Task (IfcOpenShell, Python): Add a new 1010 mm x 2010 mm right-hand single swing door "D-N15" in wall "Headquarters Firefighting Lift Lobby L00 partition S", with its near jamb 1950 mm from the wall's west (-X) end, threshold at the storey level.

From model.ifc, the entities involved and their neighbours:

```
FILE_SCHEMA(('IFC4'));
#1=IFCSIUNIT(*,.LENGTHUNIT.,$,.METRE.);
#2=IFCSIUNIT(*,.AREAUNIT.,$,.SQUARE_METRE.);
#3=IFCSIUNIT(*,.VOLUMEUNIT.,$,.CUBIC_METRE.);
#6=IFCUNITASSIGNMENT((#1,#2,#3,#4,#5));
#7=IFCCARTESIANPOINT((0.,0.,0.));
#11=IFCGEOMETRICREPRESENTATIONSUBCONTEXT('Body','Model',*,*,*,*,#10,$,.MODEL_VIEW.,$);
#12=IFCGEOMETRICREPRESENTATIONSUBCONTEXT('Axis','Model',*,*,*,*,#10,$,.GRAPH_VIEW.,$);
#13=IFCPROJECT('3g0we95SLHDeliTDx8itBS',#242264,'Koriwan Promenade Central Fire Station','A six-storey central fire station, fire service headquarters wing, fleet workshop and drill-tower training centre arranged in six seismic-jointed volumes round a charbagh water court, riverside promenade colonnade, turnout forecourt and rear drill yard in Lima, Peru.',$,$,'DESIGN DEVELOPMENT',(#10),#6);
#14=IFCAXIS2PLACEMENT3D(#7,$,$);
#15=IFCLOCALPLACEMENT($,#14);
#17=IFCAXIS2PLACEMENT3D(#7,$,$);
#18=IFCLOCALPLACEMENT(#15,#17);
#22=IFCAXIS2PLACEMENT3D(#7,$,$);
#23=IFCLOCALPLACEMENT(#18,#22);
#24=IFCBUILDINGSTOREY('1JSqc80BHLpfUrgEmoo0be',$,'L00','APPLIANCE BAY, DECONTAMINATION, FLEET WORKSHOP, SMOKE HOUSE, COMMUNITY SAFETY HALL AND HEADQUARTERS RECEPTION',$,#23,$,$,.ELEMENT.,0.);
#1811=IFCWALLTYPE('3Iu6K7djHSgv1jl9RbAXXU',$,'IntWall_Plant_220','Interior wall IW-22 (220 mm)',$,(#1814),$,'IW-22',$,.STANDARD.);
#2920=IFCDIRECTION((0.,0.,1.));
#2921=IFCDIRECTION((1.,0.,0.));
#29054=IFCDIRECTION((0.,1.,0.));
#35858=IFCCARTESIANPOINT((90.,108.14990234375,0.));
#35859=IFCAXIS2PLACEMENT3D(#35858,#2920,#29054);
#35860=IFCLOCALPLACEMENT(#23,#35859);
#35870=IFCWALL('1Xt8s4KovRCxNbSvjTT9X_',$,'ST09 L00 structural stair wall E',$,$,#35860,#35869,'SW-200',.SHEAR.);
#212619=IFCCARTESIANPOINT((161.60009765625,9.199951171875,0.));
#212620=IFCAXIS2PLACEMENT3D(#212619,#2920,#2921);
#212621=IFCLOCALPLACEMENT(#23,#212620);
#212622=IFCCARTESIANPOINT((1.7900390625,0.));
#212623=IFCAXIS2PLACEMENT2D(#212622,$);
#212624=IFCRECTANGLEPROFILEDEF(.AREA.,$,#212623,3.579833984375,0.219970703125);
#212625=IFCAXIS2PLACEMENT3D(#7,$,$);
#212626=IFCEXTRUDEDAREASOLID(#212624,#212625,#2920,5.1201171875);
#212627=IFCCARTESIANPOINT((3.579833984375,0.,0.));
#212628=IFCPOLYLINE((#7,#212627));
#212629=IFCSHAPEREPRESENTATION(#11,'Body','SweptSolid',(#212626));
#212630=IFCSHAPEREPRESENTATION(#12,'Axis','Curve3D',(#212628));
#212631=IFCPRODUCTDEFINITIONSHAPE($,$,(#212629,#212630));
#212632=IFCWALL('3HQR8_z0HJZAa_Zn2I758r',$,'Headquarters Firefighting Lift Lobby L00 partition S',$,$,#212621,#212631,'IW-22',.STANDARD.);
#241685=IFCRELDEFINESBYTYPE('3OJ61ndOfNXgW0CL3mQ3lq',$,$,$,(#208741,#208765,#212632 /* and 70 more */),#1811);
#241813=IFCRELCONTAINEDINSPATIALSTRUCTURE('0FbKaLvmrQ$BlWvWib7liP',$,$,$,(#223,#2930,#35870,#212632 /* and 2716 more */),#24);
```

```python
import numpy as np
import ifcopenshell
import ifcopenshell.api.feature
import ifcopenshell.api.geometry
import ifcopenshell.api.root
import ifcopenshell.api.spatial
import ifcopenshell.geom
import ifcopenshell.util.element
import ifcopenshell.util.placement
import ifcopenshell.util.representation
import ifcopenshell.util.shape
import ifcopenshell.util.unit

model = ifcopenshell.open("model.ifc")
unit_scale = ifcopenshell.util.unit.calculate_unit_scale(model)
settings = ifcopenshell.geom.settings()


def volume(element):
    """Net volume in cubic metres, openings subtracted."""
    shape = ifcopenshell.geom.create_shape(settings, element)
    return ifcopenshell.util.shape.get_volume(shape.geometry)


wall = model.by_guid("3HQR8_z0HJZAa_Zn2I758r")
storey = ifcopenshell.util.element.get_container(wall, ifc_class="IfcBuildingStorey")
context = ifcopenshell.util.representation.get_context(model, "Model", "Body", "MODEL_VIEW")
before = volume(wall)

width, height, from_end, sill = 1.01, 2.01, 1.95, 0.0  # metres

# The wall runs along its own X axis, and the end named is its -X end.
wall_shape = ifcopenshell.geom.create_shape(settings, wall)
x, y, z = ifcopenshell.util.shape.get_vertices(wall_shape.geometry).T
start = x.min() + from_end
face, thickness = float(y.min()), float(y.max() - y.min())
wall_matrix = ifcopenshell.util.placement.get_local_placement(wall.ObjectPlacement)
level = ifcopenshell.util.placement.get_local_placement(storey.ObjectPlacement)[2, 3]


def in_wall(x, y):
    """Placement at x, y metres in the wall's axes, at sill height."""
    matrix = wall_matrix.copy()
    matrix[:, 3] = wall_matrix @ np.array([x / unit_scale, y / unit_scale, 0.0, 1.0])
    matrix[2, 3] = level + sill / unit_scale
    return matrix


# Opening: a box that overshoots both wall faces by 50 mm.
opening = ifcopenshell.api.root.create_entity(model, ifc_class="IfcOpeningElement", predefined_type="OPENING")
box = ifcopenshell.api.geometry.add_wall_representation(
    model, context=context, length=width, height=height, thickness=thickness + 0.1
)
ifcopenshell.api.geometry.assign_representation(model, product=opening, representation=box)
ifcopenshell.api.geometry.edit_object_placement(model, product=opening, matrix=in_wall(start, face - 0.05), is_si=False)
ifcopenshell.api.feature.add_feature(model, feature=opening, element=wall)

door = ifcopenshell.api.root.create_entity(model, ifc_class="IfcDoor", name="D-N15", predefined_type="DOOR")
door.OverallWidth, door.OverallHeight = width / unit_scale, height / unit_scale
door.OperationType = "SINGLE_SWING_RIGHT"
body = ifcopenshell.api.geometry.add_door_representation(
    model,
    context=context,
    overall_width=door.OverallWidth,
    overall_height=door.OverallHeight,
    operation_type="SINGLE_SWING_RIGHT",
    lining_properties={"LiningDepth": thickness / unit_scale, "ThresholdDepth": thickness / unit_scale},
)
ifcopenshell.api.geometry.assign_representation(model, product=door, representation=body)
ifcopenshell.api.spatial.assign_container(model, products=[door], relating_structure=storey)
ifcopenshell.api.feature.add_filling(model, opening=opening, element=door)

# The lining spans the wall, so the door starts at the wall face.
ifcopenshell.api.geometry.edit_object_placement(model, product=door, matrix=in_wall(start, face), is_si=False)

after = volume(wall)

print(f"wall volume {before:.3f} -> {after:.3f} m3")

model.write("model-out.ifc")
```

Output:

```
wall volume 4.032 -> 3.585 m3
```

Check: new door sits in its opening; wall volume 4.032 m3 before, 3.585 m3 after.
